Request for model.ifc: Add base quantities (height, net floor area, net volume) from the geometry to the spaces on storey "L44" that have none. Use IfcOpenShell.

First a look at what the model holds.

```python
import ifcopenshell
import ifcopenshell.util.element
import ifcopenshell.util.unit

model = ifcopenshell.open("model.ifc")
print(model.schema)
for unit_type in ("LENGTHUNIT", "AREAUNIT", "VOLUMEUNIT"):
    print(unit_type, ifcopenshell.util.unit.calculate_unit_scale(model, unit_type))
storey = next(s for s in model.by_type("IfcBuildingStorey") if s.Name == "L44")
spaces = [e for e in ifcopenshell.util.element.get_decomposition(storey) if e.is_a("IfcSpace")]
for e in sorted(spaces, key=lambda e: e.id()):
    print(e.id(), e.is_a(), e.Name, list(ifcopenshell.util.element.get_psets(e, qtos_only=True)), sep=" | ")
```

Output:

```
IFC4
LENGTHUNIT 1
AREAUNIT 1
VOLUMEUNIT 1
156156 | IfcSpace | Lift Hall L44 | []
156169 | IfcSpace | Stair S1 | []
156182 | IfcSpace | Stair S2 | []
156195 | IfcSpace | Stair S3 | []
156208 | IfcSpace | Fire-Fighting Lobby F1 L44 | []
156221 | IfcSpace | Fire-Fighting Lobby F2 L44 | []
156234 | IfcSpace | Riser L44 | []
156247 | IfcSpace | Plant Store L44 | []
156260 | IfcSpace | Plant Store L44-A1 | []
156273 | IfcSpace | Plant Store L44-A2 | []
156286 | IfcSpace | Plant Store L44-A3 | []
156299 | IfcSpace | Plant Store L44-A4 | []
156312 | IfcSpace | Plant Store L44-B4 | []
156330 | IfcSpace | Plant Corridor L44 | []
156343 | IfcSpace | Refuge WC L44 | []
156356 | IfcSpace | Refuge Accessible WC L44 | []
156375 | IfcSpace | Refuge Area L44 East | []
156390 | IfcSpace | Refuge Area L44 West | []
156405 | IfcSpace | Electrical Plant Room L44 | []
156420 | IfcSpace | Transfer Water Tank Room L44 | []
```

```python
import ifcopenshell
import ifcopenshell.api.pset
import ifcopenshell.geom
import ifcopenshell.util.element
import ifcopenshell.util.shape
import ifcopenshell.util.unit

model = ifcopenshell.open("model.ifc")
unit_scale = ifcopenshell.util.unit.calculate_unit_scale(model)
area_scale = ifcopenshell.util.unit.calculate_unit_scale(model, "AREAUNIT")
volume_scale = ifcopenshell.util.unit.calculate_unit_scale(model, "VOLUMEUNIT")
settings = ifcopenshell.geom.settings()

storey = next(s for s in model.by_type("IfcBuildingStorey") if s.Name == "L44")
spaces = [e for e in ifcopenshell.util.element.get_decomposition(storey) if e.is_a("IfcSpace")]

for e in sorted(spaces, key=lambda e: e.id()):
    if ifcopenshell.util.element.get_psets(e, qtos_only=True, should_inherit=False):
        continue
    # Geometry comes back in metres, in the element's own axes.
    shape = ifcopenshell.geom.create_shape(settings, e)
    values = {
        "Height": ifcopenshell.util.shape.get_z(shape.geometry) / unit_scale,
        "NetFloorArea": ifcopenshell.util.shape.get_footprint_area(shape.geometry) / area_scale,
        "NetVolume": ifcopenshell.util.shape.get_volume(shape.geometry) / volume_scale,
    }
    qto = ifcopenshell.api.pset.add_qto(model, product=e, name="Qto_SpaceBaseQuantities")
    ifcopenshell.api.pset.edit_qto(model, qto=qto, properties=values)
    print(e.id(), {k: round(v, 3) for k, v in values.items()})

model.write("model-out.ifc")
```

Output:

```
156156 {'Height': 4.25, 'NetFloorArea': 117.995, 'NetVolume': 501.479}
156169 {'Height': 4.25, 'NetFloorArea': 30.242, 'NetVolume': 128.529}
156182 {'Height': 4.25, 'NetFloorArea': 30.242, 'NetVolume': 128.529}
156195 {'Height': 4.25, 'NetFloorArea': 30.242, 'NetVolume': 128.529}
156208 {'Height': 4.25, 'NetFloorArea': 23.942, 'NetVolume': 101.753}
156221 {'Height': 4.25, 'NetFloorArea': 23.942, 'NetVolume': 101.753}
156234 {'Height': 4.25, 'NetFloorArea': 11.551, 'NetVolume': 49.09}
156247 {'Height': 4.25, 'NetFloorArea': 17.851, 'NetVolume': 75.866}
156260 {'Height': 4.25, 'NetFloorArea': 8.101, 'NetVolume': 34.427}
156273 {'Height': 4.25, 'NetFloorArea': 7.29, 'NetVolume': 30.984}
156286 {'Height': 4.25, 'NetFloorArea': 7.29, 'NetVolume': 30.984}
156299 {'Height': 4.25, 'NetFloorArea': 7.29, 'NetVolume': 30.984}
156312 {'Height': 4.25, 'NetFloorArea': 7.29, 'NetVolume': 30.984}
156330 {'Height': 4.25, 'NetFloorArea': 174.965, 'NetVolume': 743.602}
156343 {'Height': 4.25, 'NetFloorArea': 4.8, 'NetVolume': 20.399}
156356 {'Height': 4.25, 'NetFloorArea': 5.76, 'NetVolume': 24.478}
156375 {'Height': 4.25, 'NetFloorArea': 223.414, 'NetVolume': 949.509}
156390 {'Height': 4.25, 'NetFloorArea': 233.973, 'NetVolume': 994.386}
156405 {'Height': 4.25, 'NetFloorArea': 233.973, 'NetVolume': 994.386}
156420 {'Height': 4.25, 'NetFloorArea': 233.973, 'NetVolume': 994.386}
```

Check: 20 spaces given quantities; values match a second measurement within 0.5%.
